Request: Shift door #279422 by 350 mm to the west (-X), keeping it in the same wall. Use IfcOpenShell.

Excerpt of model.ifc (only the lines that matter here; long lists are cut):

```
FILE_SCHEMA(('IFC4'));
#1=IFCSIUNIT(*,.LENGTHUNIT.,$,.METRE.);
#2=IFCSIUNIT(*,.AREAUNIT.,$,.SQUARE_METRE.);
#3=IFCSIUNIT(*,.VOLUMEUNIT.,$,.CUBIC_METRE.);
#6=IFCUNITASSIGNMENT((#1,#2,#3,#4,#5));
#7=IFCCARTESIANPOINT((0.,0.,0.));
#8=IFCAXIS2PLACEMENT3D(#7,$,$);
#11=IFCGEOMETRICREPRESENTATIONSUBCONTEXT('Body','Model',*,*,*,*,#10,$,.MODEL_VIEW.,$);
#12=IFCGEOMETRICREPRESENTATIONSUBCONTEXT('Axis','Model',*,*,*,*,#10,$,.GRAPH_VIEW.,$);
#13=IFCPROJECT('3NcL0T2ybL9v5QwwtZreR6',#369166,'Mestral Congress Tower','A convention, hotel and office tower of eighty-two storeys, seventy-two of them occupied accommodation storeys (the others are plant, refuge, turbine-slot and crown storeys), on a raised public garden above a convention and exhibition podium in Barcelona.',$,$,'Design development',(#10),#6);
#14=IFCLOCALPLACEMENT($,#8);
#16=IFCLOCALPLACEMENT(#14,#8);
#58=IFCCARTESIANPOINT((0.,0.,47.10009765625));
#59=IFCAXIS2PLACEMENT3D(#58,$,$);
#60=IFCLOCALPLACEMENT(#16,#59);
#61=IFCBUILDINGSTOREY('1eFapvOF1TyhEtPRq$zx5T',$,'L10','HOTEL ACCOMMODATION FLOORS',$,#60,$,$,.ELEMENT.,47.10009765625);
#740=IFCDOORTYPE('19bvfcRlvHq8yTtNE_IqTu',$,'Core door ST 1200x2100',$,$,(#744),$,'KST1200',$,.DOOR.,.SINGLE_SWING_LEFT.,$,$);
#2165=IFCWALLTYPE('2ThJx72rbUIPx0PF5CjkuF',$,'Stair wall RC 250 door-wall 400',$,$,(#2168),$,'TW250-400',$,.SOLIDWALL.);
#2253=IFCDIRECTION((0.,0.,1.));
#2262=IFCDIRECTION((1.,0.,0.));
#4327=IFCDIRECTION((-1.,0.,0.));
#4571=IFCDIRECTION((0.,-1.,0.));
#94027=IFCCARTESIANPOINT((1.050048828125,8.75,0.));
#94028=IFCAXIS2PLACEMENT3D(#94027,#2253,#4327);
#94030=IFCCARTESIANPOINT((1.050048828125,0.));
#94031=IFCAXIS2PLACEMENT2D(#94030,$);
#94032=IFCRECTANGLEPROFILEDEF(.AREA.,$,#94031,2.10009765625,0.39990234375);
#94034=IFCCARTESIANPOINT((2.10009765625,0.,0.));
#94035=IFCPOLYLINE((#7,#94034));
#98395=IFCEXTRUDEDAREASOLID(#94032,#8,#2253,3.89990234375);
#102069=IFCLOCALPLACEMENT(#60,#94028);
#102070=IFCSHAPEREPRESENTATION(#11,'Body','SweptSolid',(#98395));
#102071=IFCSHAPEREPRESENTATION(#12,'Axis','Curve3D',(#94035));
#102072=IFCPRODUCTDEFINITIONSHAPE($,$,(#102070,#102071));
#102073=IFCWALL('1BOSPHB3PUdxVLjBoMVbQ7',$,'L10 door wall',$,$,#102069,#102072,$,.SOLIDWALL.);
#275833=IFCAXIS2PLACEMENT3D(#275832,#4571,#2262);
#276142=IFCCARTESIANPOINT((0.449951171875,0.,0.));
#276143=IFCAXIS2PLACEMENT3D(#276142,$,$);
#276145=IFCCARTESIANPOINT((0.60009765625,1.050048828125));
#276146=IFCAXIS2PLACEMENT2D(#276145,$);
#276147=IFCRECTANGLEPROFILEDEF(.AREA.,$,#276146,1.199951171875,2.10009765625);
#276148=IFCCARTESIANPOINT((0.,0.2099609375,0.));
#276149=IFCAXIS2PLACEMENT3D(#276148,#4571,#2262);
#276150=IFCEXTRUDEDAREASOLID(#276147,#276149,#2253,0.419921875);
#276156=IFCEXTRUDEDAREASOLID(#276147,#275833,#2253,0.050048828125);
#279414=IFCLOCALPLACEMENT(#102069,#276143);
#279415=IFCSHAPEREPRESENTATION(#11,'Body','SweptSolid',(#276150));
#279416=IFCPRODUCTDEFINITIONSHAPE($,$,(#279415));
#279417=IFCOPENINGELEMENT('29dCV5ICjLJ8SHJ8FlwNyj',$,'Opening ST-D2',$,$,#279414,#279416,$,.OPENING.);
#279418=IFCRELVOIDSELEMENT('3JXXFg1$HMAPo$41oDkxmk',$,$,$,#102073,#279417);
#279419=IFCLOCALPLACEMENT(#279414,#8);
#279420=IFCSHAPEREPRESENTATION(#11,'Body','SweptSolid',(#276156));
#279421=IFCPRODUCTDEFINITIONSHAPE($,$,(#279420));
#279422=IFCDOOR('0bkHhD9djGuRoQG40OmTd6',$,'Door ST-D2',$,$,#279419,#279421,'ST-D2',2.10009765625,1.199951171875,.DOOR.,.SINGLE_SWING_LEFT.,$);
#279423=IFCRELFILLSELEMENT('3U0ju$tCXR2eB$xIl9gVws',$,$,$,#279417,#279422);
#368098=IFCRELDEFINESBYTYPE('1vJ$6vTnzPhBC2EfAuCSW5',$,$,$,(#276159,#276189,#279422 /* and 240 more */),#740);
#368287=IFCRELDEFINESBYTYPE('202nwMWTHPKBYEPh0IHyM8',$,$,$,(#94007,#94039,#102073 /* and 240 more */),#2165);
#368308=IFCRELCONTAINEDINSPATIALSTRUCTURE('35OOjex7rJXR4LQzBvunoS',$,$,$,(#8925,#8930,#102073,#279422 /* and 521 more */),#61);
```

```python
import ifcopenshell
import ifcopenshell.api.geometry
import ifcopenshell.util.placement

model = ifcopenshell.open("model.ifc")

door = model.by_guid("0bkHhD9djGuRoQG40OmTd6")
opening = door.FillsVoids[0].RelatingOpeningElement
wall = opening.VoidsElements[0].RelatingBuildingElement

wall_matrix = ifcopenshell.util.placement.get_local_placement(wall.ObjectPlacement)
shift = wall_matrix[:3, 0] * 0.35
before = ifcopenshell.util.placement.get_local_placement(door.ObjectPlacement)[:3, 3].copy()

# The door is placed relative to its opening, so it follows when the opening moves.
matrix = ifcopenshell.util.placement.get_local_placement(opening.ObjectPlacement)
matrix[:3, 3] += shift
ifcopenshell.api.geometry.edit_object_placement(
    model, product=opening, matrix=matrix, is_si=False, should_transform_children=True
)

after = ifcopenshell.util.placement.get_local_placement(door.ObjectPlacement)[:3, 3]
print("door moved by", (after - before).round(3) + 0.0)

model.write("model_edited.ifc")
```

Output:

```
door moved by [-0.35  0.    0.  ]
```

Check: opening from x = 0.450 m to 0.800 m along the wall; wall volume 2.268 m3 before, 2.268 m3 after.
